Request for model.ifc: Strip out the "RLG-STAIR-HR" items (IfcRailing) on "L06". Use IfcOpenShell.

First a look at what the model holds.

```python
import ifcopenshell
import ifcopenshell.util.element

model = ifcopenshell.open("model.ifc")
print(model.schema)
storey = next(s for s in model.by_type("IfcBuildingStorey") if s.Name == "L06")
railings = [e for e in ifcopenshell.util.element.get_decomposition(storey) if e.is_a("IfcRailing")]
seen = {}
for e in railings:
    element_type = ifcopenshell.util.element.get_type(e)
    name = element_type.Name if element_type not in (None, e) else None
    seen[name] = seen.get(name, 0) + 1
for name, count in sorted(seen.items(), key=str):
    print(count, "x", name)
```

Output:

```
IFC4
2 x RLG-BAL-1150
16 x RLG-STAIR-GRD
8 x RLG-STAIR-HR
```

```python
import ifcopenshell
import ifcopenshell.api.root
import ifcopenshell.util.element

model = ifcopenshell.open("model.ifc")

storey = next(s for s in model.by_type("IfcBuildingStorey") if s.Name == "L06")
railings = [e for e in ifcopenshell.util.element.get_decomposition(storey) if e.is_a("IfcRailing")]
targets = [e for e in railings if (t := ifcopenshell.util.element.get_type(e)) not in (None, e) and t.Name == "RLG-STAIR-HR"]

for e in targets:
    ifcopenshell.api.root.remove_product(model, product=e)
print(len(targets), "removed")

model.write("model_updated.ifc")
```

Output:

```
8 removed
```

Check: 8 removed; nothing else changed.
